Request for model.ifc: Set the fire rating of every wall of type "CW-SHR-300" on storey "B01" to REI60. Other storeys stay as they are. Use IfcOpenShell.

First a look at what the model holds.

```python
import ifcopenshell
import ifcopenshell.util.element

model = ifcopenshell.open("model.ifc")
print(model.schema)
storey = next(s for s in model.by_type("IfcBuildingStorey") if s.Name == "B01")
walls = [e for e in ifcopenshell.util.element.get_decomposition(storey) if e.is_a("IfcWall")]
seen = {}
for e in walls:
    element_type = ifcopenshell.util.element.get_type(e)
    key = (element_type.Name if element_type != e and element_type else None, ifcopenshell.util.element.get_pset(e, "Pset_WallCommon", "FireRating"))
    seen[key] = seen.get(key, 0) + 1
for (name, value), count in sorted(seen.items(), key=str):
    print(count, "x", name, "|", value)
```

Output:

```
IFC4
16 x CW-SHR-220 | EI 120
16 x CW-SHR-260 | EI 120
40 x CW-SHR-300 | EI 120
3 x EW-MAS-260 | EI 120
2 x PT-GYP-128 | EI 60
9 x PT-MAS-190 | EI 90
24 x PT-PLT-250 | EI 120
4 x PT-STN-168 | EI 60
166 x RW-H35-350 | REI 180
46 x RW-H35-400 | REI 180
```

```python
import ifcopenshell
import ifcopenshell.api.pset
import ifcopenshell.util.element

model = ifcopenshell.open("model.ifc")

storey = next(s for s in model.by_type("IfcBuildingStorey") if s.Name == "B01")
walls = [e for e in ifcopenshell.util.element.get_decomposition(storey) if e.is_a("IfcWall")]

count = 0
for e in walls:
    element_type = ifcopenshell.util.element.get_type(e)
    if element_type in (None, e) or element_type.Name != "CW-SHR-300":
        continue
    # add_pset returns the element's existing set when there is one.
    pset = ifcopenshell.api.pset.add_pset(model, product=e, name="Pset_WallCommon")
    ifcopenshell.api.pset.edit_pset(model, pset=pset, properties={"FireRating": "REI60"})
    count += 1

print(count, "walls updated")

model.write("model_edited.ifc")
```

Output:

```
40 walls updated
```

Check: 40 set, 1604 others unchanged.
